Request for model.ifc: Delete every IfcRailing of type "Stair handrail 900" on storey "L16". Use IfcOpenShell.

First a look at what the model holds.

```python
import ifcopenshell
import ifcopenshell.util.element

model = ifcopenshell.open("model.ifc")
print(model.schema)
storey = next(s for s in model.by_type("IfcBuildingStorey") if s.Name == "L16")
railings = [e for e in ifcopenshell.util.element.get_decomposition(storey) if e.is_a("IfcRailing")]
seen = {}
for e in railings:
    element_type = ifcopenshell.util.element.get_type(e)
    name = element_type.Name if element_type not in (None, e) else None
    seen[name] = seen.get(name, 0) + 1
for name, count in sorted(seen.items(), key=str):
    print(count, "x", name)
```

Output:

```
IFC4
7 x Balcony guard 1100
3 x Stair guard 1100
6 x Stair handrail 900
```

```python
import ifcopenshell
import ifcopenshell.api.root
import ifcopenshell.util.element

model = ifcopenshell.open("model.ifc")

storey = next(s for s in model.by_type("IfcBuildingStorey") if s.Name == "L16")
railings = [e for e in ifcopenshell.util.element.get_decomposition(storey) if e.is_a("IfcRailing")]
targets = [e for e in railings if (t := ifcopenshell.util.element.get_type(e)) not in (None, e) and t.Name == "Stair handrail 900"]

for e in targets:
    ifcopenshell.api.root.remove_product(model, product=e)
print(len(targets), "removed")

model.write("model-out.ifc")
```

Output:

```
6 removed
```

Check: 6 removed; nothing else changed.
